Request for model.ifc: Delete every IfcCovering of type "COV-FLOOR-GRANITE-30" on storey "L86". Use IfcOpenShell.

First a look at what the model holds.

```python
import ifcopenshell
import ifcopenshell.util.element

model = ifcopenshell.open("model.ifc")
print(model.schema)
storey = next(s for s in model.by_type("IfcBuildingStorey") if s.Name == "L86")
coverings = [e for e in ifcopenshell.util.element.get_decomposition(storey) if e.is_a("IfcCovering")]
seen = {}
for e in coverings:
    element_type = ifcopenshell.util.element.get_type(e)
    name = element_type.Name if element_type not in (None, e) else None
    seen[name] = seen.get(name, 0) + 1
for name, count in sorted(seen.items(), key=str):
    print(count, "x", name)
```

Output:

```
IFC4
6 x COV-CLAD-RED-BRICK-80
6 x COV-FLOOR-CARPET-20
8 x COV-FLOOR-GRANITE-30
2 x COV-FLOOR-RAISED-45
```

```python
import ifcopenshell
import ifcopenshell.api.root
import ifcopenshell.util.element

model = ifcopenshell.open("model.ifc")

storey = next(s for s in model.by_type("IfcBuildingStorey") if s.Name == "L86")
coverings = [e for e in ifcopenshell.util.element.get_decomposition(storey) if e.is_a("IfcCovering")]
targets = [e for e in coverings if (t := ifcopenshell.util.element.get_type(e)) not in (None, e) and t.Name == "COV-FLOOR-GRANITE-30"]

for e in targets:
    ifcopenshell.api.root.remove_product(model, product=e)
print(len(targets), "removed")

model.write("model-out.ifc")
```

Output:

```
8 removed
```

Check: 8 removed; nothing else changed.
